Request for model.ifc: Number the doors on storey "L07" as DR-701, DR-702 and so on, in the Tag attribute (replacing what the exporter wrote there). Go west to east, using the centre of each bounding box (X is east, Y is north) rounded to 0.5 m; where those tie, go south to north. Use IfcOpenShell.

First a look at what the model holds.

```python
import ifcopenshell
import ifcopenshell.util.element
import ifcopenshell.util.placement

model = ifcopenshell.open("model.ifc")
print(model.schema)
storey = next(s for s in model.by_type("IfcBuildingStorey") if s.Name == "L07")
doors = [e for e in ifcopenshell.util.element.get_decomposition(storey) if e.is_a("IfcDoor")]
for e in sorted(doors, key=lambda e: e.id()):
    origin = ifcopenshell.util.placement.get_local_placement(e.ObjectPlacement)[:3, 3]
    print(e.id(), e.Tag, e.Name, origin.round(2) + 0.0, sep=" | ")
```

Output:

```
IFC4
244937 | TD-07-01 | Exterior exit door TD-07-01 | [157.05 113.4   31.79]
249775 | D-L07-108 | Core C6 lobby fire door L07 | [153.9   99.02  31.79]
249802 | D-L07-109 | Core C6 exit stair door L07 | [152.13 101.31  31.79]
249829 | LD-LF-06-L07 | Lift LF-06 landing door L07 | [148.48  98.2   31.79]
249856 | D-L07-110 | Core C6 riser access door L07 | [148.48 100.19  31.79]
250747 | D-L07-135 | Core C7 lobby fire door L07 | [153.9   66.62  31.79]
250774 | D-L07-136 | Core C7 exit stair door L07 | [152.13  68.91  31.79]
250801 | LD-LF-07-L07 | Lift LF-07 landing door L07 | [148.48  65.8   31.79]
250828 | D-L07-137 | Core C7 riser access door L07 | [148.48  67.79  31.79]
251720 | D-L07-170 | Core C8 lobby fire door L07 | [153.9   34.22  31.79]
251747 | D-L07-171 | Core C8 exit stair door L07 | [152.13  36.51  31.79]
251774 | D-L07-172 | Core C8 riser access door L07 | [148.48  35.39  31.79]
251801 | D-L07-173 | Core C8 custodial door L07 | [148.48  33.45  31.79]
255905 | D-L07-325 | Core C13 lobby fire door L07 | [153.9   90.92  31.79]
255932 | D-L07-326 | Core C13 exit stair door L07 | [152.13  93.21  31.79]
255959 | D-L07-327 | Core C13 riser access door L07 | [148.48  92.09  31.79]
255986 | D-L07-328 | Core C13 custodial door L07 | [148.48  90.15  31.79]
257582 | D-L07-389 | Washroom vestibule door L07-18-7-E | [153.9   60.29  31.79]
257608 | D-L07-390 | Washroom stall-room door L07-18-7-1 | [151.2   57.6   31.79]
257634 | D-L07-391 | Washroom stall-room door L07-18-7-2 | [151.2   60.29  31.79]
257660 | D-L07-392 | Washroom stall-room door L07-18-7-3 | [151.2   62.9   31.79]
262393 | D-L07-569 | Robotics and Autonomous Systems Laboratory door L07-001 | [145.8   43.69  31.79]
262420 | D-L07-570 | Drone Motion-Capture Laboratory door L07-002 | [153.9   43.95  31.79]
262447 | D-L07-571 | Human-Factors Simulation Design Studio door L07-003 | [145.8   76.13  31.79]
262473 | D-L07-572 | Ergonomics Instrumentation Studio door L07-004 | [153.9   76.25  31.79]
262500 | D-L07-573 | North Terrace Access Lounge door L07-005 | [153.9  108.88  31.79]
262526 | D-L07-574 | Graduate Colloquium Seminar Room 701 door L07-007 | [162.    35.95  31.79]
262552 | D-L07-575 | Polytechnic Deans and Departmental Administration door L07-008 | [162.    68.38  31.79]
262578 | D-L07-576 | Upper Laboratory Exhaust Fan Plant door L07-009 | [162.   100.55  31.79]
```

```python
import ifcopenshell
import ifcopenshell.geom
import ifcopenshell.util.element
import ifcopenshell.util.shape

model = ifcopenshell.open("model.ifc")
settings = ifcopenshell.geom.settings()
settings.set("use-world-coords", True)


def centre(element):
    shape = ifcopenshell.geom.create_shape(settings, element)
    return ifcopenshell.util.shape.get_bbox_centroid(shape.geometry)


storey = next(s for s in model.by_type("IfcBuildingStorey") if s.Name == "L07")
doors = [e for e in ifcopenshell.util.element.get_decomposition(storey) if e.is_a("IfcDoor")]

# Insertion points can sit at a corner or the storey origin, so sort by the geometry (in metres).
centres = {e: centre(e) for e in doors}
doors.sort(key=lambda e: (round(centres[e][0] / 0.5), centres[e][1]))

for i, e in enumerate(doors, start=1):
    number = f"DR-7{i:02d}"
    e.Tag = number
    print(e.id(), number)

model.write("model_edited.ifc")
```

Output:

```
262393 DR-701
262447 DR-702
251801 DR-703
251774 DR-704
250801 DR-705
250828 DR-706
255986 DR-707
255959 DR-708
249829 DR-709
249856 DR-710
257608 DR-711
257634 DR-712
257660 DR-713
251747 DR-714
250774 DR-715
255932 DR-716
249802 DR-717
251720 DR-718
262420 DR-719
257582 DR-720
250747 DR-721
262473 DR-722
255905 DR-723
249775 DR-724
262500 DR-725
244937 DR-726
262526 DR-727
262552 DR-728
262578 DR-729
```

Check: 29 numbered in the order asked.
